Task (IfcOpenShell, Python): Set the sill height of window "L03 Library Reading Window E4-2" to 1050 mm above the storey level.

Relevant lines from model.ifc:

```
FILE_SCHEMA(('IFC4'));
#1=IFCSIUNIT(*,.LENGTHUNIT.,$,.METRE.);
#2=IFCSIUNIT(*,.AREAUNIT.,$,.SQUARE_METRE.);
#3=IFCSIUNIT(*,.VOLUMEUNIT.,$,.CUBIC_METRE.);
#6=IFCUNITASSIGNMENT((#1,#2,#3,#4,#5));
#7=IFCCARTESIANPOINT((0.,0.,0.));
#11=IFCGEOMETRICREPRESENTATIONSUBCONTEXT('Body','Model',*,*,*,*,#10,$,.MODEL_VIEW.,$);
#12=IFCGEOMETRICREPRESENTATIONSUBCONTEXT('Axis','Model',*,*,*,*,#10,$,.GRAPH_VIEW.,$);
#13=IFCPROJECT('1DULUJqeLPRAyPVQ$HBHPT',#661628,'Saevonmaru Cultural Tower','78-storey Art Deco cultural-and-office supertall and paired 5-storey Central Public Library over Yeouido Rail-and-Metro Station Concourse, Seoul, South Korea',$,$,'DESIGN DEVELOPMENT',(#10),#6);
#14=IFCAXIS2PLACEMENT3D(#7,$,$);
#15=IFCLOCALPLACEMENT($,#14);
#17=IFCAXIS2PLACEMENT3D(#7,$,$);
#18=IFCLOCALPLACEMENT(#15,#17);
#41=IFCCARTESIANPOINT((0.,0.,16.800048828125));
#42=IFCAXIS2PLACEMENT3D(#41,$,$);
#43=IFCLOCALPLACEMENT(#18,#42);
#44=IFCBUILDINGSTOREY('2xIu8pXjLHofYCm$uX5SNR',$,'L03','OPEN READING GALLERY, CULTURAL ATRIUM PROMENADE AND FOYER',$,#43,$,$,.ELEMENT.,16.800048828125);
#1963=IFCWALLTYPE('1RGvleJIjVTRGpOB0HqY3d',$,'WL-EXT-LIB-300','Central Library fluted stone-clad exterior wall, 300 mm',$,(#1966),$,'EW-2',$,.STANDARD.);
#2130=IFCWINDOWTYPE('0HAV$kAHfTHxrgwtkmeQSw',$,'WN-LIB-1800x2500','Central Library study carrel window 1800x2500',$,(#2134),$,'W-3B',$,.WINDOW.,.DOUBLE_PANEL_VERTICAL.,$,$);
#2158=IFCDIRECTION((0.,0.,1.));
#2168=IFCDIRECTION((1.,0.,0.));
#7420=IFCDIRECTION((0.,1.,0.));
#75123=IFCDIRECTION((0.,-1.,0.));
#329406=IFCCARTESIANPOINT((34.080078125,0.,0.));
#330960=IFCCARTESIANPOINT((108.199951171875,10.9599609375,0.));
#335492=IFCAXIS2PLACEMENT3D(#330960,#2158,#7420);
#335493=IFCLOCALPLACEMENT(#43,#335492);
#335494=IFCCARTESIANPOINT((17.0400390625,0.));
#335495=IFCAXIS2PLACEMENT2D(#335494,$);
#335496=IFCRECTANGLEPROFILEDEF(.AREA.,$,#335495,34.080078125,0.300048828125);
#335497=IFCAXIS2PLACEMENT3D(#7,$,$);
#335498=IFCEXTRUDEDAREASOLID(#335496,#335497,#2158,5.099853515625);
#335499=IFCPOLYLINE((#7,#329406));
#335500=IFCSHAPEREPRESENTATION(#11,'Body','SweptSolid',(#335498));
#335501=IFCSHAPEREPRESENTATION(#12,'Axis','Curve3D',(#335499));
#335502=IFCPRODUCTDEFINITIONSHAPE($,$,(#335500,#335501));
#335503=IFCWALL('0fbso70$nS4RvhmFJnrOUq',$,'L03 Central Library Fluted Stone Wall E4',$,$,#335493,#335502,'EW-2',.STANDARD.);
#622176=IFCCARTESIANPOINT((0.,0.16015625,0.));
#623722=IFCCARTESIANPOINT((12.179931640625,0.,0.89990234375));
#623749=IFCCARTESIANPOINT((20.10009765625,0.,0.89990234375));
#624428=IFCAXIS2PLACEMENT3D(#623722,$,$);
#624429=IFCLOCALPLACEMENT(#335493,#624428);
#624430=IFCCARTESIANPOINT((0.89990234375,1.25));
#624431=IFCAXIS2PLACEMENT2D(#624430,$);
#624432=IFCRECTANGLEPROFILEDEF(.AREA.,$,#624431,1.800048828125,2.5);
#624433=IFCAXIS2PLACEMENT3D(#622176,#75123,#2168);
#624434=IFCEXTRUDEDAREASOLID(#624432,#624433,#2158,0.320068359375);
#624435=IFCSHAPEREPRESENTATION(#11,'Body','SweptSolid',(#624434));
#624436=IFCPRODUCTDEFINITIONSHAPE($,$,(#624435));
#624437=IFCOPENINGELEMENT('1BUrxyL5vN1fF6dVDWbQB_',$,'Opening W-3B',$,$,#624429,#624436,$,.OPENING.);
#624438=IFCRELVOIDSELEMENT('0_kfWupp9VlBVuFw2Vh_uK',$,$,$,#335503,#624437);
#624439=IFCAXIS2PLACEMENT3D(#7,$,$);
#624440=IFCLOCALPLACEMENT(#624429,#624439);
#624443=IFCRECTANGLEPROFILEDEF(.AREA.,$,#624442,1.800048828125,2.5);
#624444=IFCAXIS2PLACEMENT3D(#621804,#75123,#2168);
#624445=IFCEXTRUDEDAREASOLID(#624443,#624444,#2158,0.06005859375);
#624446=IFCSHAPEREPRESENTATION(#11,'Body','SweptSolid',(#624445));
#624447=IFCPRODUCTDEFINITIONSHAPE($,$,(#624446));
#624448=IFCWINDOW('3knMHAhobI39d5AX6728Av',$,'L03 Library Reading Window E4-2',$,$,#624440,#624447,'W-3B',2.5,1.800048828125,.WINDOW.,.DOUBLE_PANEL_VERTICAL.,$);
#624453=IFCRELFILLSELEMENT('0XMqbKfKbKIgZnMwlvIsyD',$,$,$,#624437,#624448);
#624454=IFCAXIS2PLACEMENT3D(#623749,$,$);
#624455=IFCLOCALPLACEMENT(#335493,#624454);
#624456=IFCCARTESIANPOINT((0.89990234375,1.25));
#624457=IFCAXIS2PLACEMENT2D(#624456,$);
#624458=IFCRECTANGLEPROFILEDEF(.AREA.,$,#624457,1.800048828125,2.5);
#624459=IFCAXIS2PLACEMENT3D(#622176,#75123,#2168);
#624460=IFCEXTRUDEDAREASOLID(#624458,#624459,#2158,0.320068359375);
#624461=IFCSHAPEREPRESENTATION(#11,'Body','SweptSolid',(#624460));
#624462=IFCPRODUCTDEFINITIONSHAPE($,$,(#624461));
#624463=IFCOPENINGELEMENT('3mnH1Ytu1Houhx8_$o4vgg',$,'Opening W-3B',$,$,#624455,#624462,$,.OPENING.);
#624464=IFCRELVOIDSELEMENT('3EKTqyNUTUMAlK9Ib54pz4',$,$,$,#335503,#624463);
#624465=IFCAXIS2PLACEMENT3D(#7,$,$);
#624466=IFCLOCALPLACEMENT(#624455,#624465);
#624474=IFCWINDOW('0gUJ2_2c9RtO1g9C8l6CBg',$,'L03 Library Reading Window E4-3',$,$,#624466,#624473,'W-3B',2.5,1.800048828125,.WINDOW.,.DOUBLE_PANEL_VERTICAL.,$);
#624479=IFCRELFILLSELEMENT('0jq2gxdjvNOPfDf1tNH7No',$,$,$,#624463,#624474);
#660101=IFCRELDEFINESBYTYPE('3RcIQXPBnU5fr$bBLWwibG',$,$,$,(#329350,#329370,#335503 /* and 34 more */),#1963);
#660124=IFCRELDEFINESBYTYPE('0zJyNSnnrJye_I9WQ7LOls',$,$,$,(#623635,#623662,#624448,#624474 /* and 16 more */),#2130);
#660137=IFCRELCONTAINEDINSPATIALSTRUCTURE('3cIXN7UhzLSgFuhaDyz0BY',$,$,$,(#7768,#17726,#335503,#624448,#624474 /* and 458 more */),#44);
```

```python
import numpy as np
import ifcopenshell
import ifcopenshell.api.geometry
import ifcopenshell.geom
import ifcopenshell.util.element
import ifcopenshell.util.placement
import ifcopenshell.util.shape
import ifcopenshell.util.unit

model = ifcopenshell.open("model.ifc")
unit_scale = ifcopenshell.util.unit.calculate_unit_scale(model)

window = model.by_guid("3knMHAhobI39d5AX6728Av")
opening = window.FillsVoids[0].RelatingOpeningElement
storey = ifcopenshell.util.element.get_container(window, ifc_class="IfcBuildingStorey")
level = ifcopenshell.util.placement.get_local_placement(storey.ObjectPlacement)[2, 3]

# The opening's origin need not be at the sill, so measure its lowest point.
shape = ifcopenshell.geom.create_shape(ifcopenshell.geom.settings(), opening)
bottom = ifcopenshell.util.shape.get_shape_bottom_elevation(shape, shape.geometry) / unit_scale
dz = level + 1.05 / unit_scale - bottom

shift = np.array([0.0, 0.0, dz])
# The window is placed relative to its opening, so it follows when the opening moves.
matrix = ifcopenshell.util.placement.get_local_placement(opening.ObjectPlacement)
matrix[:3, 3] += shift
ifcopenshell.api.geometry.edit_object_placement(
    model, product=opening, matrix=matrix, is_si=False, should_transform_children=True
)

print(f"moved by {dz * unit_scale:+.3f} m")

model.write("model_edited.ifc")
```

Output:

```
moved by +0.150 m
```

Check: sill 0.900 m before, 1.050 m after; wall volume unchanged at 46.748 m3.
